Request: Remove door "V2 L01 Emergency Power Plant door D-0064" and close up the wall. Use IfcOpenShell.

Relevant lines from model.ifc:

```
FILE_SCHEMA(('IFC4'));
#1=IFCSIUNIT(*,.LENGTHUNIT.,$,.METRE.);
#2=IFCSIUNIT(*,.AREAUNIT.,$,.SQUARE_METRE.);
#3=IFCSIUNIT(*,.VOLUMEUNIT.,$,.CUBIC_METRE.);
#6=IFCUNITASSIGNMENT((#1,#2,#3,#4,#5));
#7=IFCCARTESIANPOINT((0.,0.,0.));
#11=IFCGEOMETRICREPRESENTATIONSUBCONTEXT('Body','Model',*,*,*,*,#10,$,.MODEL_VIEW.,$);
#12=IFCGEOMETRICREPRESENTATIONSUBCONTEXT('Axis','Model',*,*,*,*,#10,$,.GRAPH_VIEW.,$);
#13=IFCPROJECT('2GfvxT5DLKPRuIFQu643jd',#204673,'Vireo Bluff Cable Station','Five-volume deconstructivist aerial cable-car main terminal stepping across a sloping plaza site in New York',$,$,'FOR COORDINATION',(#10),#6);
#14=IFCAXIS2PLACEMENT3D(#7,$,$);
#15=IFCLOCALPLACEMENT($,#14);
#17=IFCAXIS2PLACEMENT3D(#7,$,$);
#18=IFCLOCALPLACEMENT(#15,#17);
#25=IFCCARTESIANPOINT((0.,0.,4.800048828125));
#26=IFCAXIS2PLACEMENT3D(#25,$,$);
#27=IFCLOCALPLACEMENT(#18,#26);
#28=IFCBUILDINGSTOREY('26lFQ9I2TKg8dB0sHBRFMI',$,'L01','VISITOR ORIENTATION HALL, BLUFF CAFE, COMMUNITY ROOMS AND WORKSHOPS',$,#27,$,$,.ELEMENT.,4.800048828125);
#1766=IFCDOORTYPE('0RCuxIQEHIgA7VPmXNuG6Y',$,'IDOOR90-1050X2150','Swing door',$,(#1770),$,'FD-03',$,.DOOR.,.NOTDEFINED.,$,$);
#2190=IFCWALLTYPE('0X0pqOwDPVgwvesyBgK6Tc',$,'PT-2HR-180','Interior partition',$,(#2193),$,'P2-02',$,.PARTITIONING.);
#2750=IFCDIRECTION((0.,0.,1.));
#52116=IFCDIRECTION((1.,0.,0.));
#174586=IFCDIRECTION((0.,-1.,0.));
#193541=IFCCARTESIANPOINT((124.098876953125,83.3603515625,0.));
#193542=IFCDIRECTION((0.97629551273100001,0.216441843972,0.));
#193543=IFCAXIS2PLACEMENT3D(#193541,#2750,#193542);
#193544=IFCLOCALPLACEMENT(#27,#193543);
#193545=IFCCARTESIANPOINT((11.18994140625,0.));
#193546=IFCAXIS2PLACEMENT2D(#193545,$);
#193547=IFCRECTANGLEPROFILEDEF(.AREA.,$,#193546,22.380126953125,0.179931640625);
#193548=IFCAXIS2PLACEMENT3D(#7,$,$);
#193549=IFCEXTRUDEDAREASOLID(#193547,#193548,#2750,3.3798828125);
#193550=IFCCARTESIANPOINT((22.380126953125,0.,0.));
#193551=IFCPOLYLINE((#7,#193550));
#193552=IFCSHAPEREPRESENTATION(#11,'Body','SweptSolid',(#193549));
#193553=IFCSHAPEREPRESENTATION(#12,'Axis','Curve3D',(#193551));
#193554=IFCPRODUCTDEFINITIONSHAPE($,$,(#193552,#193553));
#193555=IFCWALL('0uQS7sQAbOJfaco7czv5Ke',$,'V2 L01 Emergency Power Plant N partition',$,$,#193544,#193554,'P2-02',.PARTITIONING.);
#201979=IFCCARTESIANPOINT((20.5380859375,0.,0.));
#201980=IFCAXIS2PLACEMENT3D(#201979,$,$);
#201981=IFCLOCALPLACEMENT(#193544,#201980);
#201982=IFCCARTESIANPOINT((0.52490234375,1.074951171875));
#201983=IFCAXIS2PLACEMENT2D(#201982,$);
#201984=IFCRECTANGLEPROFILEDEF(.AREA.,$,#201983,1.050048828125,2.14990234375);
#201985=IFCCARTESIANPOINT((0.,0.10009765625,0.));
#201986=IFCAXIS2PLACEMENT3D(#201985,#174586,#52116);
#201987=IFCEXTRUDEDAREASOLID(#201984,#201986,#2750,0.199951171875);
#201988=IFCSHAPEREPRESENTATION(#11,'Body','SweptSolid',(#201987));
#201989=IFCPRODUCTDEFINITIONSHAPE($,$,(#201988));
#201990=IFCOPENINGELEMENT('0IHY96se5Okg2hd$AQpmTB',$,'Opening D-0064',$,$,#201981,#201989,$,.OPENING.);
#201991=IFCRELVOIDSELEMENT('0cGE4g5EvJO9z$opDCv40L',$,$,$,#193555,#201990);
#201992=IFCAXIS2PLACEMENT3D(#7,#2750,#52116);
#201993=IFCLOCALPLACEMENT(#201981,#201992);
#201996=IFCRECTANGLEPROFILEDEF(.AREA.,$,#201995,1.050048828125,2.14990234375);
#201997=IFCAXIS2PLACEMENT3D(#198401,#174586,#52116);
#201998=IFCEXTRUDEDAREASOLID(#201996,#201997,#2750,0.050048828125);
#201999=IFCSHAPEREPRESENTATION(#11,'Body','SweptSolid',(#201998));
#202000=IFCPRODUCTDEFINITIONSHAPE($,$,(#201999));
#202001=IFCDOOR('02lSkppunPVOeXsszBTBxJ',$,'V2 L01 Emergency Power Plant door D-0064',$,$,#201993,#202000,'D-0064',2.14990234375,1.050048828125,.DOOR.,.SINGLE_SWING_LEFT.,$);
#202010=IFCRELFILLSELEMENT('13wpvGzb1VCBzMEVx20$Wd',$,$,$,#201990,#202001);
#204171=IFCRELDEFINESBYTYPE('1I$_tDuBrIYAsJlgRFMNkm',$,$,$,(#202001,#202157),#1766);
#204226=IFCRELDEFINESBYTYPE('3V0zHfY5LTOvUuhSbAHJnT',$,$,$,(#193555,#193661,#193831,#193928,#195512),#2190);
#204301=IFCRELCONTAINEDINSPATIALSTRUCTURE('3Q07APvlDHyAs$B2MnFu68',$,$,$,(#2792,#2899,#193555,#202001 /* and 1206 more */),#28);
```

```python
import ifcopenshell
import ifcopenshell.api.feature
import ifcopenshell.api.root
import ifcopenshell.geom
import ifcopenshell.util.shape

model = ifcopenshell.open("model.ifc")
settings = ifcopenshell.geom.settings()


def volume(element):
    """Net volume in cubic metres, openings subtracted."""
    shape = ifcopenshell.geom.create_shape(settings, element)
    return ifcopenshell.util.shape.get_volume(shape.geometry)


door = model.by_id(202001)
opening = door.FillsVoids[0].RelatingOpeningElement
wall = opening.VoidsElements[0].RelatingBuildingElement
before = volume(wall)

ifcopenshell.api.root.remove_product(model, product=door)
ifcopenshell.api.feature.remove_feature(model, feature=opening)

after = volume(wall)

print(f"wall volume {before:.3f} -> {after:.3f} m3")

model.write("model-out.ifc")
```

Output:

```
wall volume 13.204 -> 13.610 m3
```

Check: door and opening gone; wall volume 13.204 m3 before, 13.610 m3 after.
